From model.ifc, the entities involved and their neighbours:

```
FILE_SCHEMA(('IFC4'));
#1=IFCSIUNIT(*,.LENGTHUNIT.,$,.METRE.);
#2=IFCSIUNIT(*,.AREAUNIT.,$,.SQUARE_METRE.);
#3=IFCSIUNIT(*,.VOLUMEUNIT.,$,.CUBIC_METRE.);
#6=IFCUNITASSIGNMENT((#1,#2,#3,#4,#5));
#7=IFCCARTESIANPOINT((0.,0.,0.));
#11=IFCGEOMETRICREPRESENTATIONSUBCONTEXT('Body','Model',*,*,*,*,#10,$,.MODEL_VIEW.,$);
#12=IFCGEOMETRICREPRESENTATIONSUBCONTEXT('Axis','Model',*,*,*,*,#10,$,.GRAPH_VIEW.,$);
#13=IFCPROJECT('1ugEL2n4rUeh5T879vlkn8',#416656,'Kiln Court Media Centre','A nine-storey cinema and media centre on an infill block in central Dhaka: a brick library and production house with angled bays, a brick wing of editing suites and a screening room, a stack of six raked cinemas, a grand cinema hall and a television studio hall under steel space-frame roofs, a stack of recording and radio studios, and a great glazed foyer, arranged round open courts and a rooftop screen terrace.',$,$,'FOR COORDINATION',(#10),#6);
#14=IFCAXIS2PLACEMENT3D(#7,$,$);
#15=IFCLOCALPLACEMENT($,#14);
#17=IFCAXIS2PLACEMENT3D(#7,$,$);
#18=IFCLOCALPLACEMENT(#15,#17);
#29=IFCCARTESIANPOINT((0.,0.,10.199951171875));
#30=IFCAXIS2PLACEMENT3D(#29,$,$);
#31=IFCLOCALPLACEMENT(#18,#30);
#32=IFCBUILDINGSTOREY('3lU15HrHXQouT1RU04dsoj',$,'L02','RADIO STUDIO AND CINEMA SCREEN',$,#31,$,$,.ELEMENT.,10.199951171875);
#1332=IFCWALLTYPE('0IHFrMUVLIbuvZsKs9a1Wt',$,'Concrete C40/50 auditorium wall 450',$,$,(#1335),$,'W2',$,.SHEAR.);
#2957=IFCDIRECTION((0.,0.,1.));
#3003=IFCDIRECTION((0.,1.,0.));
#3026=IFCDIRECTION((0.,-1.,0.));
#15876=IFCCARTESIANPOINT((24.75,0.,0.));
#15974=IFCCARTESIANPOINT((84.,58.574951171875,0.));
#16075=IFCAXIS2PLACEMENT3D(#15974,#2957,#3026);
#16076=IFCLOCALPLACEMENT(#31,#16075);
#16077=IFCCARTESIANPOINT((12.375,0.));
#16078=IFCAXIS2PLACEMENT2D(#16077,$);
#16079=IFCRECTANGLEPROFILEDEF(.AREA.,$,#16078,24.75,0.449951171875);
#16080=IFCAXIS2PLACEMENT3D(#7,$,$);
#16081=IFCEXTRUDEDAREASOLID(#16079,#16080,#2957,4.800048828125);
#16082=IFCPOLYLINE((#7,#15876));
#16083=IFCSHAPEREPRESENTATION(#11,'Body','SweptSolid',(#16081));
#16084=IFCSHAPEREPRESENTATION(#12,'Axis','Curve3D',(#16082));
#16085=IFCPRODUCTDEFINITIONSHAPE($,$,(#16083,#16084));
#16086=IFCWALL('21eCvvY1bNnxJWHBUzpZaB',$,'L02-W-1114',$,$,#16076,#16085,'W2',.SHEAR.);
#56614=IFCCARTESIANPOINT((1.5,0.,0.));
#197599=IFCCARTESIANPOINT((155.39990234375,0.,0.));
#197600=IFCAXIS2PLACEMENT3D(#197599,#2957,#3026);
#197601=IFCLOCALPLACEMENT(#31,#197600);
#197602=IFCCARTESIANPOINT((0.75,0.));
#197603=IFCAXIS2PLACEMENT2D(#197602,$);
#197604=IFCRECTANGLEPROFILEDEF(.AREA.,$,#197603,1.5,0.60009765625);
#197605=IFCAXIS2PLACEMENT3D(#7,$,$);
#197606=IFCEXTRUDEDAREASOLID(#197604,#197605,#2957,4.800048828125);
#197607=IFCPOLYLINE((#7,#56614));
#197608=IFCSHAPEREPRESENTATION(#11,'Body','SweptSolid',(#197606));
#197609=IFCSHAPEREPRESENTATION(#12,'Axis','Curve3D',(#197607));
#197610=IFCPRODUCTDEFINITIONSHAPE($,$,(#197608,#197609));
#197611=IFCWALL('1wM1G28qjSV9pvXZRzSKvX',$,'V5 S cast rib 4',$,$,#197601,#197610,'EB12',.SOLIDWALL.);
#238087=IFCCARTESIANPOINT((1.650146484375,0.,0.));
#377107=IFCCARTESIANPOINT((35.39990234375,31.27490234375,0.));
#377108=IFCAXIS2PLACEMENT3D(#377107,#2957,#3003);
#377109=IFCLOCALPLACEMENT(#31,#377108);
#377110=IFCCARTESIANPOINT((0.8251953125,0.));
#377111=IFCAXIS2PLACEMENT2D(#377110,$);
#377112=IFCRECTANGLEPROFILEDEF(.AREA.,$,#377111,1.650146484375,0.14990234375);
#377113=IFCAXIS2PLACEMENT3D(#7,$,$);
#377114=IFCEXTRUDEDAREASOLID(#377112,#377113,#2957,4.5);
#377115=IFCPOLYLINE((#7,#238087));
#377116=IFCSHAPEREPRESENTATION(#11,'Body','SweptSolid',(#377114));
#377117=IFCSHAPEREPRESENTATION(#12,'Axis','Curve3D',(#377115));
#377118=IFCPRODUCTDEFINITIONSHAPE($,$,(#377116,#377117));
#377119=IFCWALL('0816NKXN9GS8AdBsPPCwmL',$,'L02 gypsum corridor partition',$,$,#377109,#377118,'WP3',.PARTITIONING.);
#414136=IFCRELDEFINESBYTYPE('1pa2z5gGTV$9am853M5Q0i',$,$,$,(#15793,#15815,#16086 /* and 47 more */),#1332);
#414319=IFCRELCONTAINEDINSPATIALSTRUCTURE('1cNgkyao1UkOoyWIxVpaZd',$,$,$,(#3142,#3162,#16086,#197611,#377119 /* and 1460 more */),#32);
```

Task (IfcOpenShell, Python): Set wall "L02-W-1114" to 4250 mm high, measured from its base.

```python
import ifcopenshell
import ifcopenshell.geom
import ifcopenshell.util.representation
import ifcopenshell.util.shape
import ifcopenshell.util.unit

model = ifcopenshell.open("model.ifc")
unit_scale = ifcopenshell.util.unit.calculate_unit_scale(model)
settings = ifcopenshell.geom.settings()


def volume(element):
    """Net volume in cubic metres, openings subtracted."""
    shape = ifcopenshell.geom.create_shape(settings, element)
    return ifcopenshell.util.shape.get_volume(shape.geometry)


wall = model.by_guid("21eCvvY1bNnxJWHBUzpZaB")
before = volume(wall)

body = ifcopenshell.util.representation.get_representation(wall, "Model", "Body")
solid = body.Items[0]
old_height = solid.Depth
solid.Depth = 4.25 / unit_scale
after = volume(wall)

print(f"height {old_height:g} -> {solid.Depth:g}, volume {before:.3f} -> {after:.3f} m3")

model.write("model-out.ifc")
```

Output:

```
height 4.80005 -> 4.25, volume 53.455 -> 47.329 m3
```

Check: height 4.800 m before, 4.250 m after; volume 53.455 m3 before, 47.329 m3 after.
